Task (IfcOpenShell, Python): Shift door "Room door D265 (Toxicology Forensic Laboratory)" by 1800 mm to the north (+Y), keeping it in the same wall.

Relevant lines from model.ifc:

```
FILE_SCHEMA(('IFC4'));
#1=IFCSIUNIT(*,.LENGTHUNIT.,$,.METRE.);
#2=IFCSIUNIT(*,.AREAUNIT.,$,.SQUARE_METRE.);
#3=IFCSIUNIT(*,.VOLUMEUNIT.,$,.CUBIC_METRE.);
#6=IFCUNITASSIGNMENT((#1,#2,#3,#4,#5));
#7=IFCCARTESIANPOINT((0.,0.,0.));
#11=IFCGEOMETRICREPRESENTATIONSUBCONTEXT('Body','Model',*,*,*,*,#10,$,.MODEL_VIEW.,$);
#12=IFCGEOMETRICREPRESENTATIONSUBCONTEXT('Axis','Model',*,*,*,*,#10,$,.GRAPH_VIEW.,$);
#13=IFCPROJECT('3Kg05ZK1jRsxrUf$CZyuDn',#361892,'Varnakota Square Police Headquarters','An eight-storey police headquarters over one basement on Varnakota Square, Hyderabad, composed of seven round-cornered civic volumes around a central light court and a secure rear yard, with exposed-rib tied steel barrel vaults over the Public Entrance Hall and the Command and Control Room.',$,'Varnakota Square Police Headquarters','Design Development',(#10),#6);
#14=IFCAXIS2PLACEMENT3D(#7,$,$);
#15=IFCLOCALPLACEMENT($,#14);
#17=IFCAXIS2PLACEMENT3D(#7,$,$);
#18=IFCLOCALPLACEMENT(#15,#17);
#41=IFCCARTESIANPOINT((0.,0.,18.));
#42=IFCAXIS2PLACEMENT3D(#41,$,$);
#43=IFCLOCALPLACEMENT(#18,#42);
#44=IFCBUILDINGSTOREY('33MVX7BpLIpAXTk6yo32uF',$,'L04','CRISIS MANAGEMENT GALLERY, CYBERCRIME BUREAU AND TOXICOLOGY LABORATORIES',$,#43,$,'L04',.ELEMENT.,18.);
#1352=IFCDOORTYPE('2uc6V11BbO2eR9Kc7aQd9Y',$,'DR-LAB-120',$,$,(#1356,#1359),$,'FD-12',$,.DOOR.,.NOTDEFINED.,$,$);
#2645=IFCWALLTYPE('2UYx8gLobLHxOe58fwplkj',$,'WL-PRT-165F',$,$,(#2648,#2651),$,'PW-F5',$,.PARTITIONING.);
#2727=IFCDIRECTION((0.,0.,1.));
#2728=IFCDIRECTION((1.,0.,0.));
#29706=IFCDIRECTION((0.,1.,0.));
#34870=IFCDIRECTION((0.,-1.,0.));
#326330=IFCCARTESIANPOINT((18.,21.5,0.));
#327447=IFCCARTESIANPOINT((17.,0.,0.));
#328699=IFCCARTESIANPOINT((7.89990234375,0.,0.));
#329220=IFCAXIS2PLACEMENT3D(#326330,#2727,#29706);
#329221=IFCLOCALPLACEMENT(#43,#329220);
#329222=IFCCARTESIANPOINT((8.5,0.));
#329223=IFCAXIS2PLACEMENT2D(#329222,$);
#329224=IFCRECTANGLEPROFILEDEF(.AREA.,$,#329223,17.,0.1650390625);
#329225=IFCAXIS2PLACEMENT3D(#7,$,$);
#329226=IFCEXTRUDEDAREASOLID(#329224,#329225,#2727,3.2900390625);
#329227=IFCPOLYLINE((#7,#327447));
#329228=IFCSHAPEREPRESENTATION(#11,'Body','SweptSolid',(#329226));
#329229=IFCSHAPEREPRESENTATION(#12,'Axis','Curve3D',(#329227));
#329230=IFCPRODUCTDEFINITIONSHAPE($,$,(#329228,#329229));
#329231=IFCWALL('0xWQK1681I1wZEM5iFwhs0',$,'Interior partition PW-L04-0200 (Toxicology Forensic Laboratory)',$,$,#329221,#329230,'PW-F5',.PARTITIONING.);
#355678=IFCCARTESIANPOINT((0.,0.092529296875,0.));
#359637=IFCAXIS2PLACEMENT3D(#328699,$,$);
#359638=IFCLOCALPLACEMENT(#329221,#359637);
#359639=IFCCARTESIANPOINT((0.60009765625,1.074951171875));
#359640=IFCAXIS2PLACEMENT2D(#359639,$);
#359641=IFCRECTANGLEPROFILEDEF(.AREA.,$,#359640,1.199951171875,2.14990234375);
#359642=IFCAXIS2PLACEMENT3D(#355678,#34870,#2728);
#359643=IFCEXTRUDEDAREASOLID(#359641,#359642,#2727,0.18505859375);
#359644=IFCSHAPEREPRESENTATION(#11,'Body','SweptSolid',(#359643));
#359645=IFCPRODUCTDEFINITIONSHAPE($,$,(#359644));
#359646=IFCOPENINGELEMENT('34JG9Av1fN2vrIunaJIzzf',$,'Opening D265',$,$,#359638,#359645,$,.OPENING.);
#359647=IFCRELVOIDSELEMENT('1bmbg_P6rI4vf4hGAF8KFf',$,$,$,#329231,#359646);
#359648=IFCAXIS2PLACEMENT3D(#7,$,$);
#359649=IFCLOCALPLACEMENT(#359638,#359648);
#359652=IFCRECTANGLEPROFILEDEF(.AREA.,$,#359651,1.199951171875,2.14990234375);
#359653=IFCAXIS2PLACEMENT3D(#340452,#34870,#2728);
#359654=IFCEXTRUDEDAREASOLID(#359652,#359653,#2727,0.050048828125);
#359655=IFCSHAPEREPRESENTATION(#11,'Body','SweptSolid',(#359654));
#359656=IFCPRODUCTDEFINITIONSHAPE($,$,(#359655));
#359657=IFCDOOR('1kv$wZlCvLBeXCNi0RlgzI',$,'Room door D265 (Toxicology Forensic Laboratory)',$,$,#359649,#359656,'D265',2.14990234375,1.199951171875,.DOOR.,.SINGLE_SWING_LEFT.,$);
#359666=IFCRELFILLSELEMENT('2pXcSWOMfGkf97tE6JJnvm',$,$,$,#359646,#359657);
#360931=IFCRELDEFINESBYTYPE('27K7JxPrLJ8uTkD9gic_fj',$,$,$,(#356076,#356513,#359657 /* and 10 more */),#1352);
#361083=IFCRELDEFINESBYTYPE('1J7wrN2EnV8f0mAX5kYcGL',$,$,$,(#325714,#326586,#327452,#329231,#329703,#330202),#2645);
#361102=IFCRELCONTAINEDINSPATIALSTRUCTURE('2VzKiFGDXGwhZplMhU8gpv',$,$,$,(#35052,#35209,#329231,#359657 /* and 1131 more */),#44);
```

```python
import ifcopenshell
import ifcopenshell.api.geometry
import ifcopenshell.util.placement

model = ifcopenshell.open("model.ifc")

door = model.by_guid("1kv$wZlCvLBeXCNi0RlgzI")
opening = door.FillsVoids[0].RelatingOpeningElement
wall = opening.VoidsElements[0].RelatingBuildingElement

wall_matrix = ifcopenshell.util.placement.get_local_placement(wall.ObjectPlacement)
shift = wall_matrix[:3, 0] * 1.8
before = ifcopenshell.util.placement.get_local_placement(door.ObjectPlacement)[:3, 3].copy()

# The door is placed relative to its opening, so it follows when the opening moves.
matrix = ifcopenshell.util.placement.get_local_placement(opening.ObjectPlacement)
matrix[:3, 3] += shift
ifcopenshell.api.geometry.edit_object_placement(
    model, product=opening, matrix=matrix, is_si=False, should_transform_children=True
)

after = ifcopenshell.util.placement.get_local_placement(door.ObjectPlacement)[:3, 3]
print("door moved by", (after - before).round(3) + 0.0)

model.write("model_updated.ifc")
```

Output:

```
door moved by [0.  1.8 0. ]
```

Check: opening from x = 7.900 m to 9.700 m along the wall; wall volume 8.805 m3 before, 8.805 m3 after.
